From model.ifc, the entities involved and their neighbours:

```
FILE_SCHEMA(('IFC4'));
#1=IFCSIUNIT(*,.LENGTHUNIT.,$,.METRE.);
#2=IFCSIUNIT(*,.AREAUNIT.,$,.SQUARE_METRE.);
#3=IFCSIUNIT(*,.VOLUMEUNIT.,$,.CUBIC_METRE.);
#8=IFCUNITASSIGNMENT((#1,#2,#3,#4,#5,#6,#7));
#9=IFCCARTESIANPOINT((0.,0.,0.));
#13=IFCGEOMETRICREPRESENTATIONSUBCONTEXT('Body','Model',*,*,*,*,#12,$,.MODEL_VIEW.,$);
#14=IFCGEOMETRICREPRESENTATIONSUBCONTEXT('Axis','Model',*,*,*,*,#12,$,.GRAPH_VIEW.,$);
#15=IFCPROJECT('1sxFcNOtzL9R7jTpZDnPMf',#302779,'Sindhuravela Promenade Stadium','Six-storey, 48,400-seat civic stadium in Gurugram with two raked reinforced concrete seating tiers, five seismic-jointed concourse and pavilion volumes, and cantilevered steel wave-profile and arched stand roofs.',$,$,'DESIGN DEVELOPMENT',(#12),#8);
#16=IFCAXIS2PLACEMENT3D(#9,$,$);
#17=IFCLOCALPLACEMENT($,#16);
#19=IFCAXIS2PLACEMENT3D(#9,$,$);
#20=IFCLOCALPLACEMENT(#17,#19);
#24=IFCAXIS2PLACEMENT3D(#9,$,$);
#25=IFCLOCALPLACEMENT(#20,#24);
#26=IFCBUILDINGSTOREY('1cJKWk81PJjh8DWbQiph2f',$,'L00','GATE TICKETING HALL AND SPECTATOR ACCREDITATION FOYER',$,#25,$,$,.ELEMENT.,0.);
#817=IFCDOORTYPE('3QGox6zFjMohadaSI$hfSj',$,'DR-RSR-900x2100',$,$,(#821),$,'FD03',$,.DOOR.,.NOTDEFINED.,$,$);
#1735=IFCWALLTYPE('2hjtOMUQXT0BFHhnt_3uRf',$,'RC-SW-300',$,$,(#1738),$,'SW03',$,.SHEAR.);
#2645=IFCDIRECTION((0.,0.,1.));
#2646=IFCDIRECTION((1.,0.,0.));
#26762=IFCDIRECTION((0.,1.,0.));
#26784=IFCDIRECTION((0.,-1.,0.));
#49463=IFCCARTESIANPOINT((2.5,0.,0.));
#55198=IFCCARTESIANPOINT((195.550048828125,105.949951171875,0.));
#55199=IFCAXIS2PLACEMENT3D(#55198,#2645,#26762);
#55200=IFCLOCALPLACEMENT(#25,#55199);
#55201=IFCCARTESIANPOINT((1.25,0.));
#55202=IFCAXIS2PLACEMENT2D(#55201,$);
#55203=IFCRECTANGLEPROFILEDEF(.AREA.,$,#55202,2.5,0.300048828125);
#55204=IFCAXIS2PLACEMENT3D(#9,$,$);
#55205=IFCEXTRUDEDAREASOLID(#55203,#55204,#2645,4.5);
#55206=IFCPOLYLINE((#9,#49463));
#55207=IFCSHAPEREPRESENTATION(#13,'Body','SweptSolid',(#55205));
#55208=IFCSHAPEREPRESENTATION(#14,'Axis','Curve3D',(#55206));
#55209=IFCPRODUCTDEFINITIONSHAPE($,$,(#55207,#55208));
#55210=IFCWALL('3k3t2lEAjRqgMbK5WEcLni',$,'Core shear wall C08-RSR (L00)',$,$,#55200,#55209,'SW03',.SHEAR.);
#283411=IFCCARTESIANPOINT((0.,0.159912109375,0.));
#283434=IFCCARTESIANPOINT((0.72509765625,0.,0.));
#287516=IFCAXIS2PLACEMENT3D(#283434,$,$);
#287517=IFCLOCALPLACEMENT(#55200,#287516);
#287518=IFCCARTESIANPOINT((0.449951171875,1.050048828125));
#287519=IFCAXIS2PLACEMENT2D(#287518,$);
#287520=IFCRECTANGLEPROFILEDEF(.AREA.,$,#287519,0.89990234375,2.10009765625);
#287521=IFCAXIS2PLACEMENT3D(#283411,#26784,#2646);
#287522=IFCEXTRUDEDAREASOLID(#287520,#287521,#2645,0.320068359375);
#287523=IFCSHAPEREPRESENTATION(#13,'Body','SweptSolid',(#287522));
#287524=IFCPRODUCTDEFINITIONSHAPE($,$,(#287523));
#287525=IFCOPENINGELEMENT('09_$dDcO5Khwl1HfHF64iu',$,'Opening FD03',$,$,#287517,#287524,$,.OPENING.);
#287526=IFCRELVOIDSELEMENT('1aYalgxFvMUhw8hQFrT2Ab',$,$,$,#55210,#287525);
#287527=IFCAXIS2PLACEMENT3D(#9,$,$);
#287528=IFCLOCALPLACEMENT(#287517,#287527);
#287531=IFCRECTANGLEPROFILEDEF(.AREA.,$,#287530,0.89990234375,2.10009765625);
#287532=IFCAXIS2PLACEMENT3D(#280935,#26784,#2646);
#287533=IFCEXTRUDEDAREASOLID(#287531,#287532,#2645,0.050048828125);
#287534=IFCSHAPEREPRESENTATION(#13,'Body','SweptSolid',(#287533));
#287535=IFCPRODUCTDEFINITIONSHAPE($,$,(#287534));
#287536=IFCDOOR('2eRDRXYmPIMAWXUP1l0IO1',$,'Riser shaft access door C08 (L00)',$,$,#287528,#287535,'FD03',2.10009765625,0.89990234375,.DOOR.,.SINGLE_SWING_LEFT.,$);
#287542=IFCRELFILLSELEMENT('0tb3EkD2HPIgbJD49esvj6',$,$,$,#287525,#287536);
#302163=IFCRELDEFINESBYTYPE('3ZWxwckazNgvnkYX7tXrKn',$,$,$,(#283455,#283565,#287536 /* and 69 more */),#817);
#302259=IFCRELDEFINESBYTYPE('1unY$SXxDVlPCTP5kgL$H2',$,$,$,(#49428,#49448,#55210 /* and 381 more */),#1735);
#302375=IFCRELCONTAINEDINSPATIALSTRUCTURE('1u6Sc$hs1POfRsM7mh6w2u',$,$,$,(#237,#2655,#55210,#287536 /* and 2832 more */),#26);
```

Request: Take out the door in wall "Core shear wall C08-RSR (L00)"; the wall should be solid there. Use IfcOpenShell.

```python
import ifcopenshell
import ifcopenshell.api.feature
import ifcopenshell.api.root
import ifcopenshell.geom
import ifcopenshell.util.shape

model = ifcopenshell.open("model.ifc")
settings = ifcopenshell.geom.settings()


def volume(element):
    """Net volume in cubic metres, openings subtracted."""
    shape = ifcopenshell.geom.create_shape(settings, element)
    return ifcopenshell.util.shape.get_volume(shape.geometry)


door = model.by_guid("2eRDRXYmPIMAWXUP1l0IO1")
opening = door.FillsVoids[0].RelatingOpeningElement
wall = opening.VoidsElements[0].RelatingBuildingElement
before = volume(wall)

ifcopenshell.api.root.remove_product(model, product=door)
ifcopenshell.api.feature.remove_feature(model, feature=opening)

after = volume(wall)

print(f"wall volume {before:.3f} -> {after:.3f} m3")

model.write("model_updated.ifc")
```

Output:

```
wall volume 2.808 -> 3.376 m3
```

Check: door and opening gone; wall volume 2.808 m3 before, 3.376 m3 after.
